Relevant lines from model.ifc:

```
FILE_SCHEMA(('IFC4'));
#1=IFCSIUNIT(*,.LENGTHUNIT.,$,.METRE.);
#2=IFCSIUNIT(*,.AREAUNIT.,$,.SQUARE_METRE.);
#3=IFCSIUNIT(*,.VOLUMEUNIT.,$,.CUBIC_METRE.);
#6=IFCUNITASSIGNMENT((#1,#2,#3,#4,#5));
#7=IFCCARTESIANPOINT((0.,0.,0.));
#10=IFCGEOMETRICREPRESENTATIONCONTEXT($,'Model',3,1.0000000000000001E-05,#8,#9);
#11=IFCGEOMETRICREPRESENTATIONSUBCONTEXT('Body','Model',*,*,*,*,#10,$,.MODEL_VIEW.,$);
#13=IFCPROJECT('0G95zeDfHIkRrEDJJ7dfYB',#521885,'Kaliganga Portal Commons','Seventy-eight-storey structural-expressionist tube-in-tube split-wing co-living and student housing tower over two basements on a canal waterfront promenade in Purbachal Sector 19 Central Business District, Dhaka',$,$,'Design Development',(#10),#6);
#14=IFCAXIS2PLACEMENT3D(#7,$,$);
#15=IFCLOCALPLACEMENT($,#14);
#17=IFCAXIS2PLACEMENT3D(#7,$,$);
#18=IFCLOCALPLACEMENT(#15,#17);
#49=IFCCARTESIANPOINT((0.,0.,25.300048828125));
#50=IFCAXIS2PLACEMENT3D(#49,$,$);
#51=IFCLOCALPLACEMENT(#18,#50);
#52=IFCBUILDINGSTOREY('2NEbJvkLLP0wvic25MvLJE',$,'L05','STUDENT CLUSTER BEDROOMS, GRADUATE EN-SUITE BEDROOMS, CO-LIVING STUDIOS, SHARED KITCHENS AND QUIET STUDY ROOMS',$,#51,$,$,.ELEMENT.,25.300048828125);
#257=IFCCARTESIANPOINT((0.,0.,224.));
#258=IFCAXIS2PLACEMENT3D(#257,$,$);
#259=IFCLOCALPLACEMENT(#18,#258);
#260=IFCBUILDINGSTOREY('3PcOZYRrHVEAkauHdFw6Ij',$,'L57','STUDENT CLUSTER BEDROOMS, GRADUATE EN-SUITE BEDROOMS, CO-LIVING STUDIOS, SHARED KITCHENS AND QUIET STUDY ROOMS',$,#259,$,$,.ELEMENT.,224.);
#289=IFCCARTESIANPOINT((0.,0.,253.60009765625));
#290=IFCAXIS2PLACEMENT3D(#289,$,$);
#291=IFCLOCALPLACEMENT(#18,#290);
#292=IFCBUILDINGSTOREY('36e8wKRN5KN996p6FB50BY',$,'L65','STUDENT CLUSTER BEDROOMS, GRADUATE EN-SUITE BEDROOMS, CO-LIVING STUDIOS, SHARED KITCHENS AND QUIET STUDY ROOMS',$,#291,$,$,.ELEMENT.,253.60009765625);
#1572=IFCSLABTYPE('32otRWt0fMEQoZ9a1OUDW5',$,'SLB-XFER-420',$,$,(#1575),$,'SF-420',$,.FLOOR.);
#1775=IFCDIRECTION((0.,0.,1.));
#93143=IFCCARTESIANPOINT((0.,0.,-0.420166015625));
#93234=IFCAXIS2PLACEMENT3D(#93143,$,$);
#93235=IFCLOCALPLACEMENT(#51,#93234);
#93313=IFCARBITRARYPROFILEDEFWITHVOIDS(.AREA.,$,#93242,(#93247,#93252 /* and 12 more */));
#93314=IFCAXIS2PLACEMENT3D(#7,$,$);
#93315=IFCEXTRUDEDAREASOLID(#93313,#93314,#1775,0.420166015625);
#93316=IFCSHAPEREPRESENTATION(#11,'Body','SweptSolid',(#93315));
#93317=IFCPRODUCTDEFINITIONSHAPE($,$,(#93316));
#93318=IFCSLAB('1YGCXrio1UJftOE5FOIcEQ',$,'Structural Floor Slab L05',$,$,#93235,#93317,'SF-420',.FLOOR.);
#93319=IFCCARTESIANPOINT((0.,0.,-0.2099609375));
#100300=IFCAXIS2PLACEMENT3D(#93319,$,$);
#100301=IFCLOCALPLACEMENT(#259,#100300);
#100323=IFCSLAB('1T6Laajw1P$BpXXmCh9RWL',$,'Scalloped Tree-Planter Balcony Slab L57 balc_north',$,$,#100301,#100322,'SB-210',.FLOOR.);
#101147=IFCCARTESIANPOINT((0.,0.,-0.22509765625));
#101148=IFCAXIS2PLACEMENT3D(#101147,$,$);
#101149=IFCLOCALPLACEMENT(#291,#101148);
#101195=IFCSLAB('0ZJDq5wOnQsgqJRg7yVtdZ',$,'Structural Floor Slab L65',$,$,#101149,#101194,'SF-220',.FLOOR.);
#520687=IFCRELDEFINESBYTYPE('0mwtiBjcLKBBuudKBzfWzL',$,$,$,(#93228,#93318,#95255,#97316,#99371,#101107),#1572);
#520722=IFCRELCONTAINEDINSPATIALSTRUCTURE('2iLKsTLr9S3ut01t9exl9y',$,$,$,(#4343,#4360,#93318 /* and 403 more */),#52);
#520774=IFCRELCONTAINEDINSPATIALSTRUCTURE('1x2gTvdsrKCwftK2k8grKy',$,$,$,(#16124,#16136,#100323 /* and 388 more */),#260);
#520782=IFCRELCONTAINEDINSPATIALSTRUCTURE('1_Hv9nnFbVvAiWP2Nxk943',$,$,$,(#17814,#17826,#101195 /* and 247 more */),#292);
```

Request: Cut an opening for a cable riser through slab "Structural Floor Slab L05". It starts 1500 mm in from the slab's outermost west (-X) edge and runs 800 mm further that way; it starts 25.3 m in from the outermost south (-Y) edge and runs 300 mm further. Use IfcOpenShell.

```python
import numpy as np
import ifcopenshell
import ifcopenshell.api.feature
import ifcopenshell.api.geometry
import ifcopenshell.api.root
import ifcopenshell.geom
import ifcopenshell.util.placement
import ifcopenshell.util.representation
import ifcopenshell.util.shape
import ifcopenshell.util.unit

model = ifcopenshell.open("model.ifc")
unit_scale = ifcopenshell.util.unit.calculate_unit_scale(model)
settings = ifcopenshell.geom.settings()


def volume(element):
    """Net volume in cubic metres, openings subtracted."""
    shape = ifcopenshell.geom.create_shape(settings, element)
    return ifcopenshell.util.shape.get_volume(shape.geometry)


slab = model.by_guid("1YGCXrio1UJftOE5FOIcEQ")
before = volume(slab)

# Extent in the slab's own axes, in metres. The edges named are its -X and -Y sides.
slab_shape = ifcopenshell.geom.create_shape(settings, slab)
vertices = ifcopenshell.util.shape.get_vertices(slab_shape.geometry)
x_min, y_min, bottom = vertices.min(axis=0)
top = vertices[:, 2].max()

opening = ifcopenshell.api.root.create_entity(model, ifc_class="IfcOpeningElement", name="Cable riser opening", predefined_type="OPENING")
context = ifcopenshell.util.representation.get_context(model, "Model", "Body", "MODEL_VIEW")
width, depth = 0.8, 0.3
outline = [(0.0, 0.0), (width, 0.0), (width, depth), (0.0, depth), (0.0, 0.0)]
# Overshoot both faces by 50 mm so the cut is clean.
shape = ifcopenshell.api.geometry.add_slab_representation(
    model, context=context, depth=top - bottom + 0.1, polyline=outline
)
ifcopenshell.api.geometry.assign_representation(model, product=opening, representation=shape)

matrix = ifcopenshell.util.placement.get_local_placement(slab.ObjectPlacement)
matrix[:, 3] = matrix @ np.append(np.array([x_min + 1.5, y_min + 25.3, bottom - 0.05]) / unit_scale, 1.0)
ifcopenshell.api.geometry.edit_object_placement(model, product=opening, matrix=matrix, is_si=False)
ifcopenshell.api.feature.add_feature(model, feature=opening, element=slab)

after = volume(slab)

print(f"slab volume {before:.3f} -> {after:.3f} m3")

model.write("model_edited.ifc")
```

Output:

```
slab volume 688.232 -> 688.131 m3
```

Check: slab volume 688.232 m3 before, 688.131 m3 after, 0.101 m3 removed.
